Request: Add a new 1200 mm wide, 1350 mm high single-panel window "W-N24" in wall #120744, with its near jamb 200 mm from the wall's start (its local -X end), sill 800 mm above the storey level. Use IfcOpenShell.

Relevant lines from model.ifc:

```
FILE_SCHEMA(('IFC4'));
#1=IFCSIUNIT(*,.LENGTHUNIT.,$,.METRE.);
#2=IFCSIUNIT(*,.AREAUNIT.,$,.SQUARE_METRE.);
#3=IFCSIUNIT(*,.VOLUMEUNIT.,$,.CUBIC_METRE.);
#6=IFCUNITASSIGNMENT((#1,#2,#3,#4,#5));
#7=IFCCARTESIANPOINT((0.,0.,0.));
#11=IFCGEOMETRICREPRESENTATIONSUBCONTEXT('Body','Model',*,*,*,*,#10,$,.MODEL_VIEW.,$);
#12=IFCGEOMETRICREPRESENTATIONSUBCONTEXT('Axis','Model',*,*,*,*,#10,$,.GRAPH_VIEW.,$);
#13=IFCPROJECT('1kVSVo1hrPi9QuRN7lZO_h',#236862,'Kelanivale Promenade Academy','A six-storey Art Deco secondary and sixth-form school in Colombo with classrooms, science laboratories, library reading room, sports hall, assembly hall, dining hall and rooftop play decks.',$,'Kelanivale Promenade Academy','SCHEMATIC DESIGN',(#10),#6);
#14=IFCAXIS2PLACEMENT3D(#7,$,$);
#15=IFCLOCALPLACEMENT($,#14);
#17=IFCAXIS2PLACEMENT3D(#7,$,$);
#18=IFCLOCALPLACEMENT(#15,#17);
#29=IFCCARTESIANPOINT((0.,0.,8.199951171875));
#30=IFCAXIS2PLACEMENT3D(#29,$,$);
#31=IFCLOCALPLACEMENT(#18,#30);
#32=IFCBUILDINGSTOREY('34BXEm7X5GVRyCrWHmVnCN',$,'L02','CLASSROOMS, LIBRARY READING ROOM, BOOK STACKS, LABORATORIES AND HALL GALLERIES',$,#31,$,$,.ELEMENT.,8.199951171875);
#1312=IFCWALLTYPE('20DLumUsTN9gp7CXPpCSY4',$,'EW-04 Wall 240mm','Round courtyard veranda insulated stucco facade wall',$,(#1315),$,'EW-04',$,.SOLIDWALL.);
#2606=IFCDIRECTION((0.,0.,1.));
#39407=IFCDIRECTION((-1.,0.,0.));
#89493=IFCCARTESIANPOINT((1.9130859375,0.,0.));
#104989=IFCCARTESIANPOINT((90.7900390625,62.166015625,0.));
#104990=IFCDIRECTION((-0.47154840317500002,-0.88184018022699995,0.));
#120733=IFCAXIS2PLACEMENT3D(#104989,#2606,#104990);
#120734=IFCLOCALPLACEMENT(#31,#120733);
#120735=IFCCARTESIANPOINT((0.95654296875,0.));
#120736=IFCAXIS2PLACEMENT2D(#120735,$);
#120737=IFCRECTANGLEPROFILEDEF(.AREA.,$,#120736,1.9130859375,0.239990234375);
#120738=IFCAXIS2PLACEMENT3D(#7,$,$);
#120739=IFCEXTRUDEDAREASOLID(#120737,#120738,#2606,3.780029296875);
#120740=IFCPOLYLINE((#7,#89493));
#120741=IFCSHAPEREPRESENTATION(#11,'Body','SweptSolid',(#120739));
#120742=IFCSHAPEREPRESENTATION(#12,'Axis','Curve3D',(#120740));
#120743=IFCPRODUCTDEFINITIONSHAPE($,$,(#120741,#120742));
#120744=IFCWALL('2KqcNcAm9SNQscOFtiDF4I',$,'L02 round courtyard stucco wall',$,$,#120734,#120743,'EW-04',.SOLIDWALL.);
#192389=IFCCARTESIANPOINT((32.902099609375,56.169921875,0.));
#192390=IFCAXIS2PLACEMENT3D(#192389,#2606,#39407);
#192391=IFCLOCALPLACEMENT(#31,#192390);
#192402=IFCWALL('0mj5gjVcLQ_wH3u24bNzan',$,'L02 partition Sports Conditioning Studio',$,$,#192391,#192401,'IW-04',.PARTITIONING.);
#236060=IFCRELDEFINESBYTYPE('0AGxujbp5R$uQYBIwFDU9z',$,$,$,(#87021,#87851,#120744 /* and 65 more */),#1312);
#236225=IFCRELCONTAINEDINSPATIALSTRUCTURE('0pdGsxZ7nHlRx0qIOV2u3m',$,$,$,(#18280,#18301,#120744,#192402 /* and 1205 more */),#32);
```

```python
import numpy as np
import ifcopenshell
import ifcopenshell.api.feature
import ifcopenshell.api.geometry
import ifcopenshell.api.root
import ifcopenshell.api.spatial
import ifcopenshell.geom
import ifcopenshell.util.element
import ifcopenshell.util.placement
import ifcopenshell.util.representation
import ifcopenshell.util.shape
import ifcopenshell.util.unit

model = ifcopenshell.open("model.ifc")
unit_scale = ifcopenshell.util.unit.calculate_unit_scale(model)
settings = ifcopenshell.geom.settings()


def volume(element):
    """Net volume in cubic metres, openings subtracted."""
    shape = ifcopenshell.geom.create_shape(settings, element)
    return ifcopenshell.util.shape.get_volume(shape.geometry)


wall = model.by_guid("2KqcNcAm9SNQscOFtiDF4I")
storey = ifcopenshell.util.element.get_container(wall, ifc_class="IfcBuildingStorey")
context = ifcopenshell.util.representation.get_context(model, "Model", "Body", "MODEL_VIEW")
before = volume(wall)

width, height, from_end, sill = 1.2, 1.35, 0.2, 0.8  # metres

# The wall runs along its own X axis, and the end named is its -X end.
wall_shape = ifcopenshell.geom.create_shape(settings, wall)
x, y, z = ifcopenshell.util.shape.get_vertices(wall_shape.geometry).T
start = x.min() + from_end
face, thickness = float(y.min()), float(y.max() - y.min())
wall_matrix = ifcopenshell.util.placement.get_local_placement(wall.ObjectPlacement)
level = ifcopenshell.util.placement.get_local_placement(storey.ObjectPlacement)[2, 3]


def in_wall(x, y):
    """Placement at x, y metres in the wall's axes, at sill height."""
    matrix = wall_matrix.copy()
    matrix[:, 3] = wall_matrix @ np.array([x / unit_scale, y / unit_scale, 0.0, 1.0])
    matrix[2, 3] = level + sill / unit_scale
    return matrix


# Opening: a box that overshoots both wall faces by 50 mm.
opening = ifcopenshell.api.root.create_entity(model, ifc_class="IfcOpeningElement", predefined_type="OPENING")
box = ifcopenshell.api.geometry.add_wall_representation(
    model, context=context, length=width, height=height, thickness=thickness + 0.1
)
ifcopenshell.api.geometry.assign_representation(model, product=opening, representation=box)
ifcopenshell.api.geometry.edit_object_placement(model, product=opening, matrix=in_wall(start, face - 0.05), is_si=False)
ifcopenshell.api.feature.add_feature(model, feature=opening, element=wall)

window = ifcopenshell.api.root.create_entity(model, ifc_class="IfcWindow", name="W-N24", predefined_type="WINDOW")
window.OverallWidth, window.OverallHeight = width / unit_scale, height / unit_scale
window.PartitioningType = "SINGLE_PANEL"
body = ifcopenshell.api.geometry.add_window_representation(
    model,
    context=context,
    overall_width=window.OverallWidth,
    overall_height=window.OverallHeight,
    partition_type="SINGLE_PANEL",
)
ifcopenshell.api.geometry.assign_representation(model, product=window, representation=body)
ifcopenshell.api.spatial.assign_container(model, products=[window], relating_structure=storey)
ifcopenshell.api.feature.add_filling(model, opening=opening, element=window)

# Centre the window in the wall's thickness.
ifcopenshell.api.geometry.edit_object_placement(model, product=window, matrix=in_wall(start, face), is_si=False)
window_shape = ifcopenshell.geom.create_shape(settings, window)
depth = ifcopenshell.util.shape.get_vertices(window_shape.geometry)[:, 1]
offset = face + thickness / 2 - (depth.min() + depth.max()) / 2
ifcopenshell.api.geometry.edit_object_placement(model, product=window, matrix=in_wall(start, offset), is_si=False)

after = volume(wall)

print(f"wall volume {before:.3f} -> {after:.3f} m3")

model.write("model-out.ifc")
```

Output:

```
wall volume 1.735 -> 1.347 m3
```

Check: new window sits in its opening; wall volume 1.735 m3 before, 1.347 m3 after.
